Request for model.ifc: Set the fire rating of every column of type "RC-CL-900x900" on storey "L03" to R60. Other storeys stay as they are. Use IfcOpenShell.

First a look at what the model holds.

```python
import ifcopenshell
import ifcopenshell.util.element

model = ifcopenshell.open("model.ifc")
print(model.schema)
storey = next(s for s in model.by_type("IfcBuildingStorey") if s.Name == "L03")
columns = [e for e in ifcopenshell.util.element.get_decomposition(storey) if e.is_a("IfcColumn")]
seen = {}
for e in columns:
    element_type = ifcopenshell.util.element.get_type(e)
    key = (element_type.Name if element_type != e and element_type else None, ifcopenshell.util.element.get_pset(e, "Pset_ColumnCommon", "FireRating"))
    seen[key] = seen.get(key, 0) + 1
for (name, value), count in sorted(seen.items(), key=str):
    print(count, "x", name, "|", value)
```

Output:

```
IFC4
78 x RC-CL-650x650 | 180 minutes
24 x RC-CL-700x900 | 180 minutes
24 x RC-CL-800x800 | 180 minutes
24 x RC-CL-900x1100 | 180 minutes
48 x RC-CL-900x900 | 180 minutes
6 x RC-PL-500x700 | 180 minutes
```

```python
import ifcopenshell
import ifcopenshell.api.pset
import ifcopenshell.util.element

model = ifcopenshell.open("model.ifc")

storey = next(s for s in model.by_type("IfcBuildingStorey") if s.Name == "L03")
columns = [e for e in ifcopenshell.util.element.get_decomposition(storey) if e.is_a("IfcColumn")]

count = 0
for e in columns:
    element_type = ifcopenshell.util.element.get_type(e)
    if element_type in (None, e) or element_type.Name != "RC-CL-900x900":
        continue
    # add_pset returns the element's existing set when there is one.
    pset = ifcopenshell.api.pset.add_pset(model, product=e, name="Pset_ColumnCommon")
    ifcopenshell.api.pset.edit_pset(model, pset=pset, properties={"FireRating": "R60"})
    count += 1

print(count, "columns updated")

model.write("model_v2.ifc")
```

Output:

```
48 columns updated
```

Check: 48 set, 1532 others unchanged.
